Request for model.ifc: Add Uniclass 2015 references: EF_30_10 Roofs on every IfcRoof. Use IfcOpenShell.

First a look at what the model holds.

```python
import ifcopenshell

model = ifcopenshell.open("model.ifc")
print(model.schema)
print("classifications:", [c.Name for c in model.by_type("IfcClassification")])
for ifc_class in ("IfcDoor", "IfcRoof", "IfcStair", "IfcWall", "IfcWindow"):
    print(ifc_class, len(model.by_type(ifc_class)))
```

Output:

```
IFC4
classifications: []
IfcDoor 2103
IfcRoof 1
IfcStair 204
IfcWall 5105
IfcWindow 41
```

```python
import ifcopenshell
import ifcopenshell.api.classification

model = ifcopenshell.open("model.ifc")

system = ifcopenshell.api.classification.add_classification(model, classification="Uniclass 2015")

codes = {
    "IfcRoof": ("EF_30_10", "Roofs"),
}
for ifc_class, (code, name) in codes.items():
    products = model.by_type(ifc_class)
    ifcopenshell.api.classification.add_reference(
        model, products=products, classification=system, identification=code, name=name
    )
    print(code, len(products))

model.write("model-out.ifc")
```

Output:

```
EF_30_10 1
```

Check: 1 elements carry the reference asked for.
